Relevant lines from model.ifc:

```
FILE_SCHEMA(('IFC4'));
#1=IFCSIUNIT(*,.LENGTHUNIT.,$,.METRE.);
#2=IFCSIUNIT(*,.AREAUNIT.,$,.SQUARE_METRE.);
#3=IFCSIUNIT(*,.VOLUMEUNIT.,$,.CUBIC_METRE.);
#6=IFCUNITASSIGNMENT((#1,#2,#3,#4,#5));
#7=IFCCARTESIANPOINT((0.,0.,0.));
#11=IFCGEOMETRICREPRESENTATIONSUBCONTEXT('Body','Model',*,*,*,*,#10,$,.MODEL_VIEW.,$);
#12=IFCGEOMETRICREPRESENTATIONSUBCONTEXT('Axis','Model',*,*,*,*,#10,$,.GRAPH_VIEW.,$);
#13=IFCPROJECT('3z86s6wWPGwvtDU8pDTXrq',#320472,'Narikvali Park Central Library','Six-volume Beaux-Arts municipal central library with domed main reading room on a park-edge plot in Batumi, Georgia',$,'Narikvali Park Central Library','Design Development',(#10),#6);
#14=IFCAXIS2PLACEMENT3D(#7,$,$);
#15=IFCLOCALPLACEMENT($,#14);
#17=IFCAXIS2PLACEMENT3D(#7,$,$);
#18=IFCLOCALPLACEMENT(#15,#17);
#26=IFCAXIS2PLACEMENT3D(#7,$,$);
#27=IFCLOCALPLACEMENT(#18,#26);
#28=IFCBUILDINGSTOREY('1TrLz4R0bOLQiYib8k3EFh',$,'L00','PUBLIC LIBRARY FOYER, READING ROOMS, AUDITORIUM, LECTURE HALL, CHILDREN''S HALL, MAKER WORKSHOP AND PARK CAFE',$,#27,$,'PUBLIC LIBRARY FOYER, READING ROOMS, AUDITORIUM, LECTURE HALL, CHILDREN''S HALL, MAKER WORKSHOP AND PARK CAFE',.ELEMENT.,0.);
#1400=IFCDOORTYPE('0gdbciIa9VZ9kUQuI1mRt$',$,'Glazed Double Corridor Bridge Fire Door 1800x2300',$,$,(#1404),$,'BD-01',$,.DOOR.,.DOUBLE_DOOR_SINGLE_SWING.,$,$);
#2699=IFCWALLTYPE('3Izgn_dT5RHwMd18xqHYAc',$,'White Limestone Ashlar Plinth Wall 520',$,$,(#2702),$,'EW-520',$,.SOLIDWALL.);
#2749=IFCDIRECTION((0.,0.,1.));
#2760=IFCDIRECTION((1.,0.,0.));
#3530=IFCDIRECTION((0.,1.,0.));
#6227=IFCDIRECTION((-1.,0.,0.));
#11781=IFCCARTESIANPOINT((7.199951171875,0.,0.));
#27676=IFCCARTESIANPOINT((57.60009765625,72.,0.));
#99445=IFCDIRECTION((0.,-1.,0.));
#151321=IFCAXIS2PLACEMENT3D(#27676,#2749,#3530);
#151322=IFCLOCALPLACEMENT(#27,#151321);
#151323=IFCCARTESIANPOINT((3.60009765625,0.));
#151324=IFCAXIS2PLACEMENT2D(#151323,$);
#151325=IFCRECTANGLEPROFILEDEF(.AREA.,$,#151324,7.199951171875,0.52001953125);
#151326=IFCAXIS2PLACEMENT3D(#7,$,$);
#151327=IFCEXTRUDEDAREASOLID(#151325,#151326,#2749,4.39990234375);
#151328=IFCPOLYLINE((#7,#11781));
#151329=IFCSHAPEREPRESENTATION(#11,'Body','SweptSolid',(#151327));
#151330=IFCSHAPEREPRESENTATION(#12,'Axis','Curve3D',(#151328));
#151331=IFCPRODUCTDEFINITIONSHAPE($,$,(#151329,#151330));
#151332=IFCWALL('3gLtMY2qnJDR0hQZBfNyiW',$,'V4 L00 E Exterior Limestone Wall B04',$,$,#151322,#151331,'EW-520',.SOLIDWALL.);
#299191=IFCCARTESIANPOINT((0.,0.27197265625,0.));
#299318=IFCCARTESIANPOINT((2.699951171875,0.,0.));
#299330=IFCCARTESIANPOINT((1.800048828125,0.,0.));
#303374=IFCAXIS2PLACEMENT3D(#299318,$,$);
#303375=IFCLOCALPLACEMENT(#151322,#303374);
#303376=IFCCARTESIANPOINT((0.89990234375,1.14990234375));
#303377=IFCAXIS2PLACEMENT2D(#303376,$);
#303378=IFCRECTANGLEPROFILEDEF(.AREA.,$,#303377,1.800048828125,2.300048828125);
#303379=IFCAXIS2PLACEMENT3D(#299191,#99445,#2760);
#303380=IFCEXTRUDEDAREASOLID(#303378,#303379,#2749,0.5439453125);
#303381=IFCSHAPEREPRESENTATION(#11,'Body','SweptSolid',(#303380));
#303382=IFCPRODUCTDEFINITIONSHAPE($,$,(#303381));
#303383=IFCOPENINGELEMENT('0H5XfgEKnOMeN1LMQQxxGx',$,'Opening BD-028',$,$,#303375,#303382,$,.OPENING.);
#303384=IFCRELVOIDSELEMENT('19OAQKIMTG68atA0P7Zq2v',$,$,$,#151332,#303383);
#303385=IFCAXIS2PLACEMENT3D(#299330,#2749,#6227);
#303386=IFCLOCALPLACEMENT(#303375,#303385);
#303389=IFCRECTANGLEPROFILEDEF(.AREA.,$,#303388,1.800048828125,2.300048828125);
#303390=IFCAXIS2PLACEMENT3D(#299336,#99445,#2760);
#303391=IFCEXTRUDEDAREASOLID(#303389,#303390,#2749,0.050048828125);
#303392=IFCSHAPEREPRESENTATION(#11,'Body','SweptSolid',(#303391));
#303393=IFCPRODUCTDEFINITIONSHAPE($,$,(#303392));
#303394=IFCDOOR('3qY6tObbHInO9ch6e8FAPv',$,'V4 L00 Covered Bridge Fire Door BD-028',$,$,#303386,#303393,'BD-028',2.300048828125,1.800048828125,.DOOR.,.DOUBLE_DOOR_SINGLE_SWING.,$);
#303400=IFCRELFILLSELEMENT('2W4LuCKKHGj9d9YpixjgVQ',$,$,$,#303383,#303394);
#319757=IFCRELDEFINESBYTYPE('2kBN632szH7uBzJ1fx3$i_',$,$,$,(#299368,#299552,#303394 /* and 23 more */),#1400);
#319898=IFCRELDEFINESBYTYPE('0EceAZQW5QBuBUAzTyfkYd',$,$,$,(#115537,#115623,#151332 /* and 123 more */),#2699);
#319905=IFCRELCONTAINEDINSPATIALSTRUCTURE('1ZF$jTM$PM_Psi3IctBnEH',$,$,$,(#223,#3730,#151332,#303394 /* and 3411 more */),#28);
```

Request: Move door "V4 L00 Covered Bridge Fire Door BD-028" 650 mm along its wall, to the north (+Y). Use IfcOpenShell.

```python
import ifcopenshell
import ifcopenshell.api.geometry
import ifcopenshell.util.placement

model = ifcopenshell.open("model.ifc")

door = model.by_guid("3qY6tObbHInO9ch6e8FAPv")
opening = door.FillsVoids[0].RelatingOpeningElement
wall = opening.VoidsElements[0].RelatingBuildingElement

wall_matrix = ifcopenshell.util.placement.get_local_placement(wall.ObjectPlacement)
shift = wall_matrix[:3, 0] * 0.65
before = ifcopenshell.util.placement.get_local_placement(door.ObjectPlacement)[:3, 3].copy()

# The door is placed relative to its opening, so it follows when the opening moves.
matrix = ifcopenshell.util.placement.get_local_placement(opening.ObjectPlacement)
matrix[:3, 3] += shift
ifcopenshell.api.geometry.edit_object_placement(
    model, product=opening, matrix=matrix, is_si=False, should_transform_children=True
)

after = ifcopenshell.util.placement.get_local_placement(door.ObjectPlacement)[:3, 3]
print("door moved by", (after - before).round(3) + 0.0)

model.write("model_rev.ifc")
```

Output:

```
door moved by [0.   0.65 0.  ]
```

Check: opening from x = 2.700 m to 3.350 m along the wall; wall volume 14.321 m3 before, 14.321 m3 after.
